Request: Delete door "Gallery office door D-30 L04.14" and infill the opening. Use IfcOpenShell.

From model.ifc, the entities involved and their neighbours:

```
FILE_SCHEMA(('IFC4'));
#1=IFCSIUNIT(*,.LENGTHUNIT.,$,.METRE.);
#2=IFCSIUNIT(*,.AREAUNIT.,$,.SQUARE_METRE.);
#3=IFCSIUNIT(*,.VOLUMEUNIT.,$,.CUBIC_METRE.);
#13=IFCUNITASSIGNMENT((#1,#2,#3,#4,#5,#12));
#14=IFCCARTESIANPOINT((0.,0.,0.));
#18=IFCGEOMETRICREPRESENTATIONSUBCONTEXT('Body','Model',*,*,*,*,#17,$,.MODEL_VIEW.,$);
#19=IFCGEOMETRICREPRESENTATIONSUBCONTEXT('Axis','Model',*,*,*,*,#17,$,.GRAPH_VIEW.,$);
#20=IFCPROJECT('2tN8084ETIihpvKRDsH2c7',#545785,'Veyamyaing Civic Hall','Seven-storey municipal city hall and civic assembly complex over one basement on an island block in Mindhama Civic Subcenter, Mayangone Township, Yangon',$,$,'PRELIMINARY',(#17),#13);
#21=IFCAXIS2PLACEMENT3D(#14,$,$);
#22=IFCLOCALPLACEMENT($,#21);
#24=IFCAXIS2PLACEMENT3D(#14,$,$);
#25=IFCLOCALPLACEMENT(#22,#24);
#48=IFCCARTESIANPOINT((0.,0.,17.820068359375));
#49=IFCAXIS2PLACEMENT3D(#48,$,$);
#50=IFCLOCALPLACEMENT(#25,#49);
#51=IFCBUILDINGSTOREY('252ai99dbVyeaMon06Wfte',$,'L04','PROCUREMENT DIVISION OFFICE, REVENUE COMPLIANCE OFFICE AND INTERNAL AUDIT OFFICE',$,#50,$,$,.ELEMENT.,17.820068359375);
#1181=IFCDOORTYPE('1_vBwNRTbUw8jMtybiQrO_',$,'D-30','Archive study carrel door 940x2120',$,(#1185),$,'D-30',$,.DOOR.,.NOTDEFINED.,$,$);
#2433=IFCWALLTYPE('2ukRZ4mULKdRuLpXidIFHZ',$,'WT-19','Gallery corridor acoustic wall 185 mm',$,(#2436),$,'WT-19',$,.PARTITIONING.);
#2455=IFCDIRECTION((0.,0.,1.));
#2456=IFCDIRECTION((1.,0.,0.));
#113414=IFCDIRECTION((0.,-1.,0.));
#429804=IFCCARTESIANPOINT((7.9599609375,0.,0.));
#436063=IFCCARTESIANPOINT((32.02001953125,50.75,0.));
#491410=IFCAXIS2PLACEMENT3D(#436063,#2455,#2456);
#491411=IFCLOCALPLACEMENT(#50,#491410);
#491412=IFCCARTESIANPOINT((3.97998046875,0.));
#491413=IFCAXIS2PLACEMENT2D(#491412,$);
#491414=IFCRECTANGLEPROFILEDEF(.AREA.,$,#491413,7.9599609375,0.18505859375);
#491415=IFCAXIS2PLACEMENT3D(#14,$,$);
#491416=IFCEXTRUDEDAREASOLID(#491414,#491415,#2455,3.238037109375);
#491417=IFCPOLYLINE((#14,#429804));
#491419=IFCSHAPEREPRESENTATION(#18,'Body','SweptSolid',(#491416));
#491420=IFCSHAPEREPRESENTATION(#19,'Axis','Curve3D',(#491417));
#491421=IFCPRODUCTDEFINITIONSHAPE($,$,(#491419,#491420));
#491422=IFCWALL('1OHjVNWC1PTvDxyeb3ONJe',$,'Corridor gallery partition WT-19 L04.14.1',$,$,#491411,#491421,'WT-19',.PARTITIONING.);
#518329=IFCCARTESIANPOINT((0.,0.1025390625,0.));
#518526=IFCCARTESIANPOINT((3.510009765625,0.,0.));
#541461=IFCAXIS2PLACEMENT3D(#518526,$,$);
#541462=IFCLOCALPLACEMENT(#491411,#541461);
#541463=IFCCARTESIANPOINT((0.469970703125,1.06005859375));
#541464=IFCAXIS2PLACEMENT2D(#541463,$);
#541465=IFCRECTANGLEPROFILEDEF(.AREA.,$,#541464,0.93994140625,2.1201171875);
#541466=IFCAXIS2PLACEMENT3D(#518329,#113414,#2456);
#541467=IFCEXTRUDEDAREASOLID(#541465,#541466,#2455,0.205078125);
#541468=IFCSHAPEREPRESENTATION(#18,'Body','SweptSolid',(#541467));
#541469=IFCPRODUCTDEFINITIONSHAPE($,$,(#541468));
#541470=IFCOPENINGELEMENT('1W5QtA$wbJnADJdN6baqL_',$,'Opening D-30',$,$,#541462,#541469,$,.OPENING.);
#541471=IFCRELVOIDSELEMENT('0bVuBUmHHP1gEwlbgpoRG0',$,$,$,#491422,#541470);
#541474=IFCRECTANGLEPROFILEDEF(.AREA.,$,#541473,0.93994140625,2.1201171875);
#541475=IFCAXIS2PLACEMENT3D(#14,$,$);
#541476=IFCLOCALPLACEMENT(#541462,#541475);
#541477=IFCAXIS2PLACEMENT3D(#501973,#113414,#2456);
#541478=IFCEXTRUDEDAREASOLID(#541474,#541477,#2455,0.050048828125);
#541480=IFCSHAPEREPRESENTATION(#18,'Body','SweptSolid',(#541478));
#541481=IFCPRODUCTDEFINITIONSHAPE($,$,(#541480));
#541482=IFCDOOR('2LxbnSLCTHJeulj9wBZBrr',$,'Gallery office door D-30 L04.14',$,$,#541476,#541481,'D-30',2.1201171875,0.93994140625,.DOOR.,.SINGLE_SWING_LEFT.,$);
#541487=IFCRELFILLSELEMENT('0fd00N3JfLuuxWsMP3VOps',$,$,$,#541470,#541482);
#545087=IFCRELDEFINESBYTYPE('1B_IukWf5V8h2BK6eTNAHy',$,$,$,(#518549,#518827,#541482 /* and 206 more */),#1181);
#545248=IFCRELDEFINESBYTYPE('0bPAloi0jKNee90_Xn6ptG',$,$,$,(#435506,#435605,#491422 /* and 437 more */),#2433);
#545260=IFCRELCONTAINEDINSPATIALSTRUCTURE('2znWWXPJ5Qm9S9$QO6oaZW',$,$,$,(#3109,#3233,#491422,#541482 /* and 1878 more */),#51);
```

```python
import ifcopenshell
import ifcopenshell.api.feature
import ifcopenshell.api.root
import ifcopenshell.geom
import ifcopenshell.util.shape

model = ifcopenshell.open("model.ifc")
settings = ifcopenshell.geom.settings()


def volume(element):
    """Net volume in cubic metres, openings subtracted."""
    shape = ifcopenshell.geom.create_shape(settings, element)
    return ifcopenshell.util.shape.get_volume(shape.geometry)


door = model.by_guid("2LxbnSLCTHJeulj9wBZBrr")
opening = door.FillsVoids[0].RelatingOpeningElement
wall = opening.VoidsElements[0].RelatingBuildingElement
before = volume(wall)

ifcopenshell.api.root.remove_product(model, product=door)
ifcopenshell.api.feature.remove_feature(model, feature=opening)

after = volume(wall)

print(f"wall volume {before:.3f} -> {after:.3f} m3")

model.write("model_updated.ifc")
```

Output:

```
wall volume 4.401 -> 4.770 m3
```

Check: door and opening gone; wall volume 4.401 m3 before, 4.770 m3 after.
